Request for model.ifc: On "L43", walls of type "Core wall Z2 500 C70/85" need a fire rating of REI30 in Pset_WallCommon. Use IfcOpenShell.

First a look at what the model holds.

```python
import ifcopenshell
import ifcopenshell.util.element

model = ifcopenshell.open("model.ifc")
print(model.schema)
storey = next(s for s in model.by_type("IfcBuildingStorey") if s.Name == "L43")
walls = [e for e in ifcopenshell.util.element.get_decomposition(storey) if e.is_a("IfcWall")]
seen = {}
for e in walls:
    element_type = ifcopenshell.util.element.get_type(e)
    key = (element_type.Name if element_type != e and element_type else None, ifcopenshell.util.element.get_pset(e, "Pset_WallCommon", "FireRating"))
    seen[key] = seen.get(key, 0) + 1
for (name, value), count in sorted(seen.items(), key=str):
    print(count, "x", name, "|", value)
```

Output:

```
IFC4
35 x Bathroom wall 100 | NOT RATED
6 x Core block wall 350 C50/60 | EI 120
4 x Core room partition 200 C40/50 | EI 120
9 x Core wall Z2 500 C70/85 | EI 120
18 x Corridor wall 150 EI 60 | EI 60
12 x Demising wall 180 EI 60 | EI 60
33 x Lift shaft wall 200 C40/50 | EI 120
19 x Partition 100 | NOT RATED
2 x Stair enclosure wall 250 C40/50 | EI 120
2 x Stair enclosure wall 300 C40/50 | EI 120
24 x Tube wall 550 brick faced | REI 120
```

```python
import ifcopenshell
import ifcopenshell.api.pset
import ifcopenshell.util.element

model = ifcopenshell.open("model.ifc")

storey = next(s for s in model.by_type("IfcBuildingStorey") if s.Name == "L43")
walls = [e for e in ifcopenshell.util.element.get_decomposition(storey) if e.is_a("IfcWall")]

count = 0
for e in walls:
    element_type = ifcopenshell.util.element.get_type(e)
    if element_type in (None, e) or element_type.Name != "Core wall Z2 500 C70/85":
        continue
    found = ifcopenshell.util.element.get_pset(e, "Pset_WallCommon", should_inherit=False)
    if found:
        pset = model.by_id(found["id"])
        if len(ifcopenshell.util.element.get_elements_by_pset(pset)) > 1:
            pset = ifcopenshell.api.pset.unshare_pset(model, products=[e], pset=pset)[0]
    else:
        pset = ifcopenshell.api.pset.add_pset(model, product=e, name="Pset_WallCommon")
    ifcopenshell.api.pset.edit_pset(model, pset=pset, properties={"FireRating": "REI30"})
    count += 1

print(count, "walls updated")

model.write("model_updated.ifc")
```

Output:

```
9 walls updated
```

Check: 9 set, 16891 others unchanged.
